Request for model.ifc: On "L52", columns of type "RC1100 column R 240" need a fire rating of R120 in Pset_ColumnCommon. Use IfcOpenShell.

First a look at what the model holds.

```python
import ifcopenshell
import ifcopenshell.util.element

model = ifcopenshell.open("model.ifc")
print(model.schema)
storey = next(s for s in model.by_type("IfcBuildingStorey") if s.Name == "L52")
columns = [e for e in ifcopenshell.util.element.get_decomposition(storey) if e.is_a("IfcColumn")]
seen = {}
for e in columns:
    element_type = ifcopenshell.util.element.get_type(e)
    key = (element_type.Name if element_type != e and element_type else None, ifcopenshell.util.element.get_pset(e, "Pset_ColumnCommon", "FireRating"))
    seen[key] = seen.get(key, 0) + 1
for (name, value), count in sorted(seen.items(), key=str):
    print(count, "x", name, "|", value)
```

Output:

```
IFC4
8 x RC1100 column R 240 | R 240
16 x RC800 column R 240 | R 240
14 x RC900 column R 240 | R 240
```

```python
import ifcopenshell
import ifcopenshell.api.pset
import ifcopenshell.util.element

model = ifcopenshell.open("model.ifc")

storey = next(s for s in model.by_type("IfcBuildingStorey") if s.Name == "L52")
columns = [e for e in ifcopenshell.util.element.get_decomposition(storey) if e.is_a("IfcColumn")]

count = 0
for e in columns:
    element_type = ifcopenshell.util.element.get_type(e)
    if element_type in (None, e) or element_type.Name != "RC1100 column R 240":
        continue
    found = ifcopenshell.util.element.get_pset(e, "Pset_ColumnCommon", should_inherit=False)
    if found:
        pset = model.by_id(found["id"])
        if len(ifcopenshell.util.element.get_elements_by_pset(pset)) > 1:
            pset = ifcopenshell.api.pset.unshare_pset(model, products=[e], pset=pset)[0]
    else:
        pset = ifcopenshell.api.pset.add_pset(model, product=e, name="Pset_ColumnCommon")
    ifcopenshell.api.pset.edit_pset(model, pset=pset, properties={"FireRating": "R120"})
    count += 1

print(count, "columns updated")

model.write("model_updated.ifc")
```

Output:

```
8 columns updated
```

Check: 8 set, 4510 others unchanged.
